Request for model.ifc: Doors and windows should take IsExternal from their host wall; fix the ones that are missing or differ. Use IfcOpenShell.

First a look at what the model holds.

```python
import ifcopenshell
import ifcopenshell.util.element

model = ifcopenshell.open("model.ifc")
print(model.schema)
seen = {}
for e in model.by_type("IfcDoor") + model.by_type("IfcWindow"):
    if not e.FillsVoids:
        continue
    host = e.FillsVoids[0].RelatingOpeningElement.VoidsElements[0].RelatingBuildingElement
    own = ifcopenshell.util.element.get_pset(e, f"Pset_{e.is_a()[3:].removesuffix('StandardCase')}Common", "IsExternal")
    wall = ifcopenshell.util.element.get_pset(host, "Pset_WallCommon", "IsExternal")
    seen[e.is_a(), own, wall] = seen.get((e.is_a(), own, wall), 0) + 1
for (cls, own, wall), count in sorted(seen.items(), key=str):
    print(count, cls, "IsExternal:", own, "| host wall:", wall)
```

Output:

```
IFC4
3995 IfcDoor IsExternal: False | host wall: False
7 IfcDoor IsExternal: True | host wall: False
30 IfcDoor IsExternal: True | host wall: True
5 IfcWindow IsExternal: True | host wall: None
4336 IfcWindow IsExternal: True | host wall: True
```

```python
import ifcopenshell
import ifcopenshell.api.pset
import ifcopenshell.util.element

model = ifcopenshell.open("model.ifc")

count = 0
for ifc_class, pset_name in (("IfcDoor", "Pset_DoorCommon"), ("IfcWindow", "Pset_WindowCommon")):
    for e in model.by_type(ifc_class):
        if not e.FillsVoids:
            continue
        host = e.FillsVoids[0].RelatingOpeningElement.VoidsElements[0].RelatingBuildingElement
        external = ifcopenshell.util.element.get_pset(host, "Pset_WallCommon", "IsExternal")
        if external is None or ifcopenshell.util.element.get_pset(e, pset_name, "IsExternal") == external:
            continue
        pset = ifcopenshell.api.pset.add_pset(model, product=e, name=pset_name)
        ifcopenshell.api.pset.edit_pset(model, pset=pset, properties={"IsExternal": external})
        count += 1

print(count, "updated")

model.write("model_updated.ifc")
```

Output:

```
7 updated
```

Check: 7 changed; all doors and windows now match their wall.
